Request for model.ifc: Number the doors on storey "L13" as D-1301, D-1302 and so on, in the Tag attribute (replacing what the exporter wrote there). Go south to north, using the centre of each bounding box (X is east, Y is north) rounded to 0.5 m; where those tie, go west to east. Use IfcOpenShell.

First a look at what the model holds.

```python
import ifcopenshell
import ifcopenshell.util.element
import ifcopenshell.util.placement

model = ifcopenshell.open("model.ifc")
print(model.schema)
storey = next(s for s in model.by_type("IfcBuildingStorey") if s.Name == "L13")
doors = [e for e in ifcopenshell.util.element.get_decomposition(storey) if e.is_a("IfcDoor")]
for e in sorted(doors, key=lambda e: e.id()):
    origin = ifcopenshell.util.placement.get_local_placement(e.ObjectPlacement)[:3, 3]
    print(e.id(), e.Tag, e.Name, origin.round(2) + 0.0, sep=" | ")
```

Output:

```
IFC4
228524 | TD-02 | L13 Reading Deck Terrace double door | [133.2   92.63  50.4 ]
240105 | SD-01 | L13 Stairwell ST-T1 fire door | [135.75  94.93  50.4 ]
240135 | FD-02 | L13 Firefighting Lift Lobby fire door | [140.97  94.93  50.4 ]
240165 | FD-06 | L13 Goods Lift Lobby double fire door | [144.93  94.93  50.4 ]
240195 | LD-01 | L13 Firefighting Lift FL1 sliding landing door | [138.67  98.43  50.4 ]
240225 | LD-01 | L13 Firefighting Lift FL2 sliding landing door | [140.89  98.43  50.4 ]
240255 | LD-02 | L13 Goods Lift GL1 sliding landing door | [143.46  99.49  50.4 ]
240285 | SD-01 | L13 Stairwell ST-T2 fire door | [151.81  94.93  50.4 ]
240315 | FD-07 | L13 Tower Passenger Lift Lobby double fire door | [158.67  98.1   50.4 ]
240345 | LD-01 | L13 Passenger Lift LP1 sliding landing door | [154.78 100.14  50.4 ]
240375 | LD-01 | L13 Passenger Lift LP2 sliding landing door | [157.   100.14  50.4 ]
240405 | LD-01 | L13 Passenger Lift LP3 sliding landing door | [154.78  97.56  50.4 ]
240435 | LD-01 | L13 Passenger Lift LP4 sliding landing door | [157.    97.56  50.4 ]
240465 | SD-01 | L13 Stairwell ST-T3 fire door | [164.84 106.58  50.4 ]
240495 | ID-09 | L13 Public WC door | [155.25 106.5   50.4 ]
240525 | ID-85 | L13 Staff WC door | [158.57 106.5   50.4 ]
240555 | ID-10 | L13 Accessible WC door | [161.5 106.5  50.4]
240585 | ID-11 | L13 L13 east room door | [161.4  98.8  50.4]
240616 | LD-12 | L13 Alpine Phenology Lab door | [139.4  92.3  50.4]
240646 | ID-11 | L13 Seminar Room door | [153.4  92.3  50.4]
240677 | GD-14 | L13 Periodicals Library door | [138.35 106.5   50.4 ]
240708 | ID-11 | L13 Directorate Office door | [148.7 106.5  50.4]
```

```python
import ifcopenshell
import ifcopenshell.geom
import ifcopenshell.util.element
import ifcopenshell.util.shape

model = ifcopenshell.open("model.ifc")
settings = ifcopenshell.geom.settings()
settings.set("use-world-coords", True)


def centre(element):
    shape = ifcopenshell.geom.create_shape(settings, element)
    return ifcopenshell.util.shape.get_bbox_centroid(shape.geometry)


storey = next(s for s in model.by_type("IfcBuildingStorey") if s.Name == "L13")
doors = [e for e in ifcopenshell.util.element.get_decomposition(storey) if e.is_a("IfcDoor")]

# Insertion points can sit at a corner or the storey origin, so sort by the geometry (in metres).
centres = {e: centre(e) for e in doors}
doors.sort(key=lambda e: (round(centres[e][1] / 0.5), centres[e][0]))

for i, e in enumerate(doors, start=1):
    number = f"D-13{i:02d}"
    e.Tag = number
    print(e.id(), number)

model.write("model-out.ifc")
```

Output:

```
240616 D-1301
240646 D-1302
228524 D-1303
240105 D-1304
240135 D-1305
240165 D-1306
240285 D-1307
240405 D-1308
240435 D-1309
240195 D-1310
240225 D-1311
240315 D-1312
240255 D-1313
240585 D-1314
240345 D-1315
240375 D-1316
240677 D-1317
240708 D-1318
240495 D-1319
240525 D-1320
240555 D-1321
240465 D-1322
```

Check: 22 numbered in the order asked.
